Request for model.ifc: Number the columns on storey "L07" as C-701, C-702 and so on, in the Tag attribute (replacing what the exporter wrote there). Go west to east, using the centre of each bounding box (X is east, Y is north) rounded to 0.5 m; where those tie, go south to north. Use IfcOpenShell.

First a look at what the model holds.

```python
import ifcopenshell
import ifcopenshell.util.element
import ifcopenshell.util.placement

model = ifcopenshell.open("model.ifc")
print(model.schema)
storey = next(s for s in model.by_type("IfcBuildingStorey") if s.Name == "L07")
columns = [e for e in ifcopenshell.util.element.get_decomposition(storey) if e.is_a("IfcColumn")]
for e in sorted(columns, key=lambda e: e.id()):
    origin = ifcopenshell.util.placement.get_local_placement(e.ObjectPlacement)[:3, 3]
    print(e.id(), e.Tag, e.Name, origin.round(2) + 0.0, sep=" | ")
```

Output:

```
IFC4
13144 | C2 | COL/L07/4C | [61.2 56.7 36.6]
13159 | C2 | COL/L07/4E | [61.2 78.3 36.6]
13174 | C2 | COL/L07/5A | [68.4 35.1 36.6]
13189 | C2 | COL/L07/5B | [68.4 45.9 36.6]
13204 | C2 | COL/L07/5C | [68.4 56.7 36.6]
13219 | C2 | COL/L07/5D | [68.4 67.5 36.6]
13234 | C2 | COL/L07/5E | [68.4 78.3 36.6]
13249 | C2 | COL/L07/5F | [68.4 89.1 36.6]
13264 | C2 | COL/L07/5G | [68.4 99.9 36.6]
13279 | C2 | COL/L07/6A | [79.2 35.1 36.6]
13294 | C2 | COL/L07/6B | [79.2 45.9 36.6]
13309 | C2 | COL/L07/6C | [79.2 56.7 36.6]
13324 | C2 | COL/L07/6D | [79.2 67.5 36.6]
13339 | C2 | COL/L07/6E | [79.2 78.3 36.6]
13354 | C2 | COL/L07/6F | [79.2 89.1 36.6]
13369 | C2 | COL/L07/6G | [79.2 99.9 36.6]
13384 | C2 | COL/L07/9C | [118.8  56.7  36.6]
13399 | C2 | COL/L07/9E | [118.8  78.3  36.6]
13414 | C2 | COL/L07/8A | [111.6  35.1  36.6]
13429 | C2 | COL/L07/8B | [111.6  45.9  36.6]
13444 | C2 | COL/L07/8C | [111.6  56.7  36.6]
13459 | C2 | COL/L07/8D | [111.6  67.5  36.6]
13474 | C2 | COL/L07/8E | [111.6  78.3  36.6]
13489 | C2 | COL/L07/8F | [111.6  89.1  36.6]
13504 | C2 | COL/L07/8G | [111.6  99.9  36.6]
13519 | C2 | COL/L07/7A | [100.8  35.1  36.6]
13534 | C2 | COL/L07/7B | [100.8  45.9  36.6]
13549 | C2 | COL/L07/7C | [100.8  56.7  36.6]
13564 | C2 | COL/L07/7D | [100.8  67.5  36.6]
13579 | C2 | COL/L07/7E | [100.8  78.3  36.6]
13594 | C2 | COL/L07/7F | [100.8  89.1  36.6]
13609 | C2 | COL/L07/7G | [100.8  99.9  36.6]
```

```python
import ifcopenshell
import ifcopenshell.geom
import ifcopenshell.util.element
import ifcopenshell.util.shape

model = ifcopenshell.open("model.ifc")
settings = ifcopenshell.geom.settings()
settings.set("use-world-coords", True)


def centre(element):
    shape = ifcopenshell.geom.create_shape(settings, element)
    return ifcopenshell.util.shape.get_bbox_centroid(shape.geometry)


storey = next(s for s in model.by_type("IfcBuildingStorey") if s.Name == "L07")
columns = [e for e in ifcopenshell.util.element.get_decomposition(storey) if e.is_a("IfcColumn")]

# Insertion points can sit at a corner or the storey origin, so sort by the geometry (in metres).
centres = {e: centre(e) for e in columns}
columns.sort(key=lambda e: (round(centres[e][0] / 0.5), centres[e][1]))

for i, e in enumerate(columns, start=1):
    number = f"C-7{i:02d}"
    e.Tag = number
    print(e.id(), number)

model.write("model_rev.ifc")
```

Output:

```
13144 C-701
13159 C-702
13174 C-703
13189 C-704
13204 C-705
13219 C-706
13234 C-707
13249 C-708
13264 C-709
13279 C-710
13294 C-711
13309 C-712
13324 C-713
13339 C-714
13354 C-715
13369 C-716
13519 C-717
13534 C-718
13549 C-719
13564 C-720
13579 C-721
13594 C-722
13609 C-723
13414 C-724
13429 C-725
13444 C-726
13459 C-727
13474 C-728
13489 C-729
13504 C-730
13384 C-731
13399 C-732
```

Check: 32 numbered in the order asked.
